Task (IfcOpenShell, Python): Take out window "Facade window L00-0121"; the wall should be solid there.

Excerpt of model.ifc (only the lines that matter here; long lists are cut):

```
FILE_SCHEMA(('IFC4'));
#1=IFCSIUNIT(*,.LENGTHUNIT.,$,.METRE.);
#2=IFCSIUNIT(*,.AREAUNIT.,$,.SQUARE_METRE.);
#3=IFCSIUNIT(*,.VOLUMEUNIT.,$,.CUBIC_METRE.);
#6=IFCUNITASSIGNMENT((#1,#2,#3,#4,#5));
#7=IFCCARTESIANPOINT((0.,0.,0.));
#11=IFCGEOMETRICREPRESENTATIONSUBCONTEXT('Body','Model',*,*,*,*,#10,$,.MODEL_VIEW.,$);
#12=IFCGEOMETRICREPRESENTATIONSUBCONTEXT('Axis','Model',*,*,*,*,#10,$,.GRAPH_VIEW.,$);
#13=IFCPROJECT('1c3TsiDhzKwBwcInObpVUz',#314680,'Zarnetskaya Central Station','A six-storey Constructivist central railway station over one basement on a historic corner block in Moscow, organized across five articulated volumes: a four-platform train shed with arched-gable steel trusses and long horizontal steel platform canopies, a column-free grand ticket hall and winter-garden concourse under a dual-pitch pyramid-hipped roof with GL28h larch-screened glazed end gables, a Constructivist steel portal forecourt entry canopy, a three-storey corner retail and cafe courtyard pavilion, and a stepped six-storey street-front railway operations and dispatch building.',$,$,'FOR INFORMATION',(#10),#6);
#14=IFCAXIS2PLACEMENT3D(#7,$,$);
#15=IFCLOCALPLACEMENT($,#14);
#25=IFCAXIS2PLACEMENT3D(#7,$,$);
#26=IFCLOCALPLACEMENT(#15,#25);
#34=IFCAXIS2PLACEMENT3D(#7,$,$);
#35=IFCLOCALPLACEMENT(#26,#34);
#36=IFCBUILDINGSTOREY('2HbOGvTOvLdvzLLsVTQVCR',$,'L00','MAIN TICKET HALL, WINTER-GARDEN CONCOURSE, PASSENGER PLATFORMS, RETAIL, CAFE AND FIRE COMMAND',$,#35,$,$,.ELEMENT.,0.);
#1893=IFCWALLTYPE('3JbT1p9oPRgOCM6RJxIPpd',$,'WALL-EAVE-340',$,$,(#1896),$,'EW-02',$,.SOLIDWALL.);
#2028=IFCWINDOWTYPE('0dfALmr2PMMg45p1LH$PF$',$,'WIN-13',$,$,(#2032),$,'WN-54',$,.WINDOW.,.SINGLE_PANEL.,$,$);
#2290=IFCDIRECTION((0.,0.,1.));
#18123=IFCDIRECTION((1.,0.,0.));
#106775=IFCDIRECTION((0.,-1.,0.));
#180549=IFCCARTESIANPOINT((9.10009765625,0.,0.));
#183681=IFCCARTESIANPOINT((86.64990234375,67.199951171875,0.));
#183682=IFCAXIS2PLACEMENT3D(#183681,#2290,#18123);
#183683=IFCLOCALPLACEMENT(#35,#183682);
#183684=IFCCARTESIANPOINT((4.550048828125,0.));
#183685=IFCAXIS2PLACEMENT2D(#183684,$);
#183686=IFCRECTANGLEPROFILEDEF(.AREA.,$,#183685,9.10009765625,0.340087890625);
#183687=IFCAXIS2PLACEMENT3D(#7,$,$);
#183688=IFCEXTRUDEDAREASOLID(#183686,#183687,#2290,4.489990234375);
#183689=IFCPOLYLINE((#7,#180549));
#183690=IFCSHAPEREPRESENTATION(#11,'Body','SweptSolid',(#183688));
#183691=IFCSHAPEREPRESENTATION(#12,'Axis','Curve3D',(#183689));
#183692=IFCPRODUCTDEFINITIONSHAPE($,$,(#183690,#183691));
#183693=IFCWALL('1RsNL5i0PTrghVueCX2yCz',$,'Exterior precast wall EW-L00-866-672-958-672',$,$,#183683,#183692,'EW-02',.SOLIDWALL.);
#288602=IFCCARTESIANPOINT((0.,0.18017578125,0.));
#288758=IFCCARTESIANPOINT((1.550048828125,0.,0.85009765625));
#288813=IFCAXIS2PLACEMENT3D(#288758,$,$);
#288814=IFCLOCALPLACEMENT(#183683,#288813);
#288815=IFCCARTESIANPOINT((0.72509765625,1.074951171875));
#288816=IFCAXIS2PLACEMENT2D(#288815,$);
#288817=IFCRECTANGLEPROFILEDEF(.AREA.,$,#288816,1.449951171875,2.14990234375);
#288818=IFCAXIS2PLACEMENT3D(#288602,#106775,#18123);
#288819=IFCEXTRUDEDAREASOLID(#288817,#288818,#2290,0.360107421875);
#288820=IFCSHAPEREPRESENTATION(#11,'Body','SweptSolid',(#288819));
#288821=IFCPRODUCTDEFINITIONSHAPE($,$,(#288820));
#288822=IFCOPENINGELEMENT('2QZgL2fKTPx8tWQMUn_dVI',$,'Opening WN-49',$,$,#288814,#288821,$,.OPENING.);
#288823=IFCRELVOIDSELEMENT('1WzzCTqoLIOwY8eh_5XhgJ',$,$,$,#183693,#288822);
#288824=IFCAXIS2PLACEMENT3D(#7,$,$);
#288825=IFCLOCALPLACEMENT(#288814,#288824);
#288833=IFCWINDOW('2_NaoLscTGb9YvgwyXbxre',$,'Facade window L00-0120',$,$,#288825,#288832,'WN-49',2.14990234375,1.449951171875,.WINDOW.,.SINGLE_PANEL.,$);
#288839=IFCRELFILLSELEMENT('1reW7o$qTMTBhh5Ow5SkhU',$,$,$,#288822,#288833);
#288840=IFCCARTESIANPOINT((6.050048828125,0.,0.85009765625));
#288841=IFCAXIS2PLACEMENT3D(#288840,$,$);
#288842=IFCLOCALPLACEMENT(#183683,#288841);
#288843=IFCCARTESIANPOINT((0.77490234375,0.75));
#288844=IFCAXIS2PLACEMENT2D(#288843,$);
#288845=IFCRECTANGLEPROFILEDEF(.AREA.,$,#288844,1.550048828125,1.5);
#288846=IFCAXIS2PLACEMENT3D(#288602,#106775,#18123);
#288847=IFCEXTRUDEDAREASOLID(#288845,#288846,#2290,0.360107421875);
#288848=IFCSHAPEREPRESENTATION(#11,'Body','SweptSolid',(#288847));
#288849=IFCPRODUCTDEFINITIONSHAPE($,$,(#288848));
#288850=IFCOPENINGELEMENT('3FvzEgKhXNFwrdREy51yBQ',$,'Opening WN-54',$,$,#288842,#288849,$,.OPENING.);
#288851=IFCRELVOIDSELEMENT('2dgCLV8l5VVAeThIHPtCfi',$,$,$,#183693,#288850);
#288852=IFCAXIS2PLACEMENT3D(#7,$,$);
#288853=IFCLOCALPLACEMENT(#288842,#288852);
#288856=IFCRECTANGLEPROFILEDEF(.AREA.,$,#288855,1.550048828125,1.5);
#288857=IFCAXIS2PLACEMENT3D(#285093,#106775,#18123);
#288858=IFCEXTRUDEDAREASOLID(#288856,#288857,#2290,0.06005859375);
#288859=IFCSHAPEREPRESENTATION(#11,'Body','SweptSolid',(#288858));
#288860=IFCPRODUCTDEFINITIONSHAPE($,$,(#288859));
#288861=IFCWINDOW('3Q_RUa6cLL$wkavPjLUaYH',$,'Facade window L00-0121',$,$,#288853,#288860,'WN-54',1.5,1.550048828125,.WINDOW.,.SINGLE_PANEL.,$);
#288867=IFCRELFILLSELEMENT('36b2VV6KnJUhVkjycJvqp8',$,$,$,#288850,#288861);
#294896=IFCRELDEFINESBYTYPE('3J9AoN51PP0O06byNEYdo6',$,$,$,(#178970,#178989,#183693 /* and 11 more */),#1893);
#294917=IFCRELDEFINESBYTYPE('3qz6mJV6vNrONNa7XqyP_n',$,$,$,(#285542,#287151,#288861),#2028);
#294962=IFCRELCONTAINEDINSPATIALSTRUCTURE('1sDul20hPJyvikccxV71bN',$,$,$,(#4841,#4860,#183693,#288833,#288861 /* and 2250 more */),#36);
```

```python
import ifcopenshell
import ifcopenshell.api.feature
import ifcopenshell.api.root
import ifcopenshell.geom
import ifcopenshell.util.shape

model = ifcopenshell.open("model.ifc")
settings = ifcopenshell.geom.settings()


def volume(element):
    """Net volume in cubic metres, openings subtracted."""
    shape = ifcopenshell.geom.create_shape(settings, element)
    return ifcopenshell.util.shape.get_volume(shape.geometry)


window = model.by_id(288861)
opening = window.FillsVoids[0].RelatingOpeningElement
wall = opening.VoidsElements[0].RelatingBuildingElement
before = volume(wall)

ifcopenshell.api.root.remove_product(model, product=window)
ifcopenshell.api.feature.remove_feature(model, feature=opening)

after = volume(wall)

print(f"wall volume {before:.3f} -> {after:.3f} m3")

model.write("model_v2.ifc")
```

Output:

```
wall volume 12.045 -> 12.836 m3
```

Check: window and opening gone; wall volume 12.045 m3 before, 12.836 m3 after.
